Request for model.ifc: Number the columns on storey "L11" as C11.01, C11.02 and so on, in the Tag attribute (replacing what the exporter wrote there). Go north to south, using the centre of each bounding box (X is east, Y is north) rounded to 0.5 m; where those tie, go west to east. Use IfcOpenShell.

First a look at what the model holds.

```python
import ifcopenshell
import ifcopenshell.util.element
import ifcopenshell.util.placement

model = ifcopenshell.open("model.ifc")
print(model.schema)
storey = next(s for s in model.by_type("IfcBuildingStorey") if s.Name == "L11")
columns = [e for e in ifcopenshell.util.element.get_decomposition(storey) if e.is_a("IfcColumn")]
for e in sorted(columns, key=lambda e: e.id()):
    origin = ifcopenshell.util.placement.get_local_placement(e.ObjectPlacement)[:3, 3]
    print(e.id(), e.Tag, e.Name, origin.round(2) + 0.0, sep=" | ")
```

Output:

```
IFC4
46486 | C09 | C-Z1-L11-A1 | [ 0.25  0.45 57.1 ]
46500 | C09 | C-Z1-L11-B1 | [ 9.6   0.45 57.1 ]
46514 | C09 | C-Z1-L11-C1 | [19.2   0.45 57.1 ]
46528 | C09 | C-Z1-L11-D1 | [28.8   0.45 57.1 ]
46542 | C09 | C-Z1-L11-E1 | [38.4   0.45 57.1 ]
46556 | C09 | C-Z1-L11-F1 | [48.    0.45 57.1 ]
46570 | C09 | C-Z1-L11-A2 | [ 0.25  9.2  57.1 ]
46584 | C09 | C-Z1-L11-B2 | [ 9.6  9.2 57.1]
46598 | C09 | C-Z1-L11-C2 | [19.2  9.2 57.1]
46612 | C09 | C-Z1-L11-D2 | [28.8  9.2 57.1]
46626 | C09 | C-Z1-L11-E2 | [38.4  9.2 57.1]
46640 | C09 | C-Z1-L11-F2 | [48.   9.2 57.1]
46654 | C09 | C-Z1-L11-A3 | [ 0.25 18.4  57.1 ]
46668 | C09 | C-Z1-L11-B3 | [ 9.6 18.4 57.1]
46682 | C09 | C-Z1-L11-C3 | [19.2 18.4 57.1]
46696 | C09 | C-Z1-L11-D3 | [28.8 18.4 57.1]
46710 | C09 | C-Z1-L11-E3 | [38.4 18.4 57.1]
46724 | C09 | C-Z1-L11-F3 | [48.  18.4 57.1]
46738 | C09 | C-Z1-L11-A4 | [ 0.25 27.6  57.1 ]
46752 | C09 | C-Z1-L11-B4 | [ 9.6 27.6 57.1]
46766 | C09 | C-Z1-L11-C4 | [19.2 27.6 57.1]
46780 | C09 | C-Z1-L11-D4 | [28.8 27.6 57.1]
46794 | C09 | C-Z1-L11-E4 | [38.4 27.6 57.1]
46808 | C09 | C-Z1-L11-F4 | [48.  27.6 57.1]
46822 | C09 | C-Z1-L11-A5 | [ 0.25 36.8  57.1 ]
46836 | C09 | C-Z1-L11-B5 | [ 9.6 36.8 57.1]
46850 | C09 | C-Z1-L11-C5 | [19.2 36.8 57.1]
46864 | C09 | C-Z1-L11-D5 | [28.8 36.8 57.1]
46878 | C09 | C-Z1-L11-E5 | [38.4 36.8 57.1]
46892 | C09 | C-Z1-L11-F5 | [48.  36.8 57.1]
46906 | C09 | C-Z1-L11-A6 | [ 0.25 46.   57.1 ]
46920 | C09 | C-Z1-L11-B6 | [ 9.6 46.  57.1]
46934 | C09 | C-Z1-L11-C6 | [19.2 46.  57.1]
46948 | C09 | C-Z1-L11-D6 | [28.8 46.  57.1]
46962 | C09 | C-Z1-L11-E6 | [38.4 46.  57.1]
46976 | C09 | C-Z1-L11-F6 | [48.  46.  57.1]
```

```python
import ifcopenshell
import ifcopenshell.geom
import ifcopenshell.util.element
import ifcopenshell.util.shape

model = ifcopenshell.open("model.ifc")
settings = ifcopenshell.geom.settings()
settings.set("use-world-coords", True)


def centre(element):
    shape = ifcopenshell.geom.create_shape(settings, element)
    return ifcopenshell.util.shape.get_bbox_centroid(shape.geometry)


storey = next(s for s in model.by_type("IfcBuildingStorey") if s.Name == "L11")
columns = [e for e in ifcopenshell.util.element.get_decomposition(storey) if e.is_a("IfcColumn")]

# Insertion points can sit at a corner or the storey origin, so sort by the geometry (in metres).
centres = {e: centre(e) for e in columns}
columns.sort(key=lambda e: (-round(centres[e][1] / 0.5), centres[e][0]))

for i, e in enumerate(columns, start=1):
    number = f"C11.{i:02d}"
    e.Tag = number
    print(e.id(), number)

model.write("model-out.ifc")
```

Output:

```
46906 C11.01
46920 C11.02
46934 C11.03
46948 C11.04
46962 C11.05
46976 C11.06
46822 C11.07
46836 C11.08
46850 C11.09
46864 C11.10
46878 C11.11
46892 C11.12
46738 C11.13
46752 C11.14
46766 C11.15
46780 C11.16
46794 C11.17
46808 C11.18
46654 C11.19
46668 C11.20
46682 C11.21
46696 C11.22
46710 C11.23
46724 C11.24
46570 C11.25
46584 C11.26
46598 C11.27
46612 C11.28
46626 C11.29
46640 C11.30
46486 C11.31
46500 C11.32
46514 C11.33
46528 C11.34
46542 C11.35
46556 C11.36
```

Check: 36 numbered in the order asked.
